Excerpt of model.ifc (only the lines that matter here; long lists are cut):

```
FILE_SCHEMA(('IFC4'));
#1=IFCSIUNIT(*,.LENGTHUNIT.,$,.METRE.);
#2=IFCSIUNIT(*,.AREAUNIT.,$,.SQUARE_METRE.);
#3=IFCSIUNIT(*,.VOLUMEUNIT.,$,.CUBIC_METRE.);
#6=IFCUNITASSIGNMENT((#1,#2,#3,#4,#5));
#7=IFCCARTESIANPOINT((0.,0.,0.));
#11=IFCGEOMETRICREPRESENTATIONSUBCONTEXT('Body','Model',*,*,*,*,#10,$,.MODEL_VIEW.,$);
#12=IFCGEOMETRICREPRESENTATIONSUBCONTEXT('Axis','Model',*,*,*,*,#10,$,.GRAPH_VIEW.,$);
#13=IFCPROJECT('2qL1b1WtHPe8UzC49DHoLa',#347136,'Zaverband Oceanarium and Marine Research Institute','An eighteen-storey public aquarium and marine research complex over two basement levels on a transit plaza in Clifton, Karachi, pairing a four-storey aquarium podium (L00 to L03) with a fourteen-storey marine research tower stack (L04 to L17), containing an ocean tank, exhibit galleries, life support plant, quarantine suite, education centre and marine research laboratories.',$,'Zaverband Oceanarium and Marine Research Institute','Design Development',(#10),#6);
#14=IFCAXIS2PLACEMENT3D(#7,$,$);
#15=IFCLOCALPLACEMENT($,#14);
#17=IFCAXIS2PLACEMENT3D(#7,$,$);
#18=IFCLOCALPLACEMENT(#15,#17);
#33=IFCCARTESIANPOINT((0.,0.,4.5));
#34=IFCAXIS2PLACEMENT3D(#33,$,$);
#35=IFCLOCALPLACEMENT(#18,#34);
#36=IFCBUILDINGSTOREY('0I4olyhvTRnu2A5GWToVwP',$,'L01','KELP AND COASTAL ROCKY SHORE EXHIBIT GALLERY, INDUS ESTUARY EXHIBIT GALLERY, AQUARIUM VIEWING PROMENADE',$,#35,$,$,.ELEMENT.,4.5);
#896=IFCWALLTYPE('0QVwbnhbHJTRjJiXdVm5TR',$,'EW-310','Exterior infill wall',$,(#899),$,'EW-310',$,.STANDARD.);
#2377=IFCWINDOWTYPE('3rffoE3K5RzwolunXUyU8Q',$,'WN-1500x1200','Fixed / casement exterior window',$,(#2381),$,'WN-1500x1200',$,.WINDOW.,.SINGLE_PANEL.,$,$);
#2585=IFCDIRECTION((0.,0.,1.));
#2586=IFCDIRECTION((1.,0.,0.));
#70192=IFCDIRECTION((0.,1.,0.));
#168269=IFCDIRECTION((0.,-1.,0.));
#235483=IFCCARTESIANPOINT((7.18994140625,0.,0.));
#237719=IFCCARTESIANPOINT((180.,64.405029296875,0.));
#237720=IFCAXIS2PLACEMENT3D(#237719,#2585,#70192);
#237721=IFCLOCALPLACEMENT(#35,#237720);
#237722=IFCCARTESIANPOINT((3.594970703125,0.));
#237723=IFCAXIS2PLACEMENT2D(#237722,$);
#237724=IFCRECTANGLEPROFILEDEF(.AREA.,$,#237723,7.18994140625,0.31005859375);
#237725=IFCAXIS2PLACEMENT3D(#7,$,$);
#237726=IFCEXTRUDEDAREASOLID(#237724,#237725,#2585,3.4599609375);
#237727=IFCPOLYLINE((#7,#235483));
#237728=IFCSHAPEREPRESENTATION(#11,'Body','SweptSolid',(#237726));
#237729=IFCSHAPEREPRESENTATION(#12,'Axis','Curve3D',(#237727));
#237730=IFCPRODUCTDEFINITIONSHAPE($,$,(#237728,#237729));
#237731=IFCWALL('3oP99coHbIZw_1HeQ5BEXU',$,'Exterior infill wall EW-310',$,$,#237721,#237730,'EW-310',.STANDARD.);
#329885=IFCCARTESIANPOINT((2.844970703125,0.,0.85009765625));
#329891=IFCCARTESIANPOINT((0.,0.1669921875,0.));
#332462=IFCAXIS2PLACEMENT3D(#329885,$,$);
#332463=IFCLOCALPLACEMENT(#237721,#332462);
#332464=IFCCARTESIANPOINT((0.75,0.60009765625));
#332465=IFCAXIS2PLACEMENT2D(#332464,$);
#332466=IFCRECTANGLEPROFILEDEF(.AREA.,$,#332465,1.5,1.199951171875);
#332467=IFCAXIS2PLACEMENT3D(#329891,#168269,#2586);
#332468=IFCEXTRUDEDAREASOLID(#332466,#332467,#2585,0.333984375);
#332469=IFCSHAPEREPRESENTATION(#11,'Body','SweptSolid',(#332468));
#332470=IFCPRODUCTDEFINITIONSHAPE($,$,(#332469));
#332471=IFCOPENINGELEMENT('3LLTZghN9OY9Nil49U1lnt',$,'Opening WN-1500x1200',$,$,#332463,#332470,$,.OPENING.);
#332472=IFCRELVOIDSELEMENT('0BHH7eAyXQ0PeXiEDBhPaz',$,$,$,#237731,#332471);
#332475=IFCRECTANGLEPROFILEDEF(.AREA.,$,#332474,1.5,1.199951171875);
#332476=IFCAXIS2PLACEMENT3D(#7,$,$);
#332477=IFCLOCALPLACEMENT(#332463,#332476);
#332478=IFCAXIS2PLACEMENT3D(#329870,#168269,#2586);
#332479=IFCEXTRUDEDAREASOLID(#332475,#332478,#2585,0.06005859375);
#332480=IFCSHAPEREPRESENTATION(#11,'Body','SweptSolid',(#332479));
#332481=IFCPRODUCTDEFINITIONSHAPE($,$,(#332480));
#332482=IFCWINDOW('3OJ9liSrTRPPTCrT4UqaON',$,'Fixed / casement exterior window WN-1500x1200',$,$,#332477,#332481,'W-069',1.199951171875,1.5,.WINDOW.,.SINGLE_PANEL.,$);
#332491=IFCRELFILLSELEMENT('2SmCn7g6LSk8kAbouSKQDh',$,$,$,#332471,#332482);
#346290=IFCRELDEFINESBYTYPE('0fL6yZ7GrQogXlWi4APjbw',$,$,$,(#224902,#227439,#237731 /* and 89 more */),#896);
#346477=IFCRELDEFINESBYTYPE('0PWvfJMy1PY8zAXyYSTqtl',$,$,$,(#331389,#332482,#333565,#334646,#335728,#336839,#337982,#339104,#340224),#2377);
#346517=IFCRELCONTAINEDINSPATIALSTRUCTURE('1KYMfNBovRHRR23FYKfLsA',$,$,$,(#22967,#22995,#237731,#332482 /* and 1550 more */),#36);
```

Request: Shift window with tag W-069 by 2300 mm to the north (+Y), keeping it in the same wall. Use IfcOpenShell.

```python
import ifcopenshell
import ifcopenshell.api.geometry
import ifcopenshell.util.placement
import ifcopenshell.util.unit

model = ifcopenshell.open("model.ifc")
unit_scale = ifcopenshell.util.unit.calculate_unit_scale(model)

window = model.by_guid("3OJ9liSrTRPPTCrT4UqaON")
opening = window.FillsVoids[0].RelatingOpeningElement
wall = opening.VoidsElements[0].RelatingBuildingElement

wall_matrix = ifcopenshell.util.placement.get_local_placement(wall.ObjectPlacement)
shift = wall_matrix[:3, 0] * 2.3 / unit_scale
before = ifcopenshell.util.placement.get_local_placement(window.ObjectPlacement)[:3, 3].copy()

# The window is placed relative to its opening, so it follows when the opening moves.
matrix = ifcopenshell.util.placement.get_local_placement(opening.ObjectPlacement)
matrix[:3, 3] += shift
ifcopenshell.api.geometry.edit_object_placement(
    model, product=opening, matrix=matrix, is_si=False, should_transform_children=True
)

after = ifcopenshell.util.placement.get_local_placement(window.ObjectPlacement)[:3, 3]
print("window moved by", (after - before).round(3) + 0.0)

model.write("model_updated.ifc")
```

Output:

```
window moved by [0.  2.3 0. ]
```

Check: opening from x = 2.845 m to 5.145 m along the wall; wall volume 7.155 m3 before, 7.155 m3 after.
